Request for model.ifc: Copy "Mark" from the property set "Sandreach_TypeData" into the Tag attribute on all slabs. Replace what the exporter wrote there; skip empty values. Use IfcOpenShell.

First a look at what the model holds.

```python
import ifcopenshell
import ifcopenshell.util.element

model = ifcopenshell.open("model.ifc")
print(model.schema)
slabs = model.by_type("IfcSlab")
print(len(slabs), "slabs")
for e in slabs[:8]:
    source = ifcopenshell.util.element.get_pset(e, "Sandreach_TypeData", "Mark")
    target = e.Tag
    print(e.id(), repr(source), repr(target), sep=" | ")
```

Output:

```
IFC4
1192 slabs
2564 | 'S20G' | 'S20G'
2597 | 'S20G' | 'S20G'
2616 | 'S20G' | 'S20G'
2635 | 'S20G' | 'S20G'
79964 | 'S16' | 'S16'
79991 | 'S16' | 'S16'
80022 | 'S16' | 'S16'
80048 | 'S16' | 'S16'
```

```python
import ifcopenshell
import ifcopenshell.util.element

model = ifcopenshell.open("model.ifc")

count = 0
for e in model.by_type("IfcSlab"):
    value = ifcopenshell.util.element.get_pset(e, "Sandreach_TypeData", "Mark")
    current = e.Tag
    if not value or not value.strip() or current == value:
        continue
    e.Tag = value
    count += 1

print(count, "slabs updated")

model.write("model-out.ifc")
```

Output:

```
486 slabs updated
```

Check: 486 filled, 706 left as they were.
